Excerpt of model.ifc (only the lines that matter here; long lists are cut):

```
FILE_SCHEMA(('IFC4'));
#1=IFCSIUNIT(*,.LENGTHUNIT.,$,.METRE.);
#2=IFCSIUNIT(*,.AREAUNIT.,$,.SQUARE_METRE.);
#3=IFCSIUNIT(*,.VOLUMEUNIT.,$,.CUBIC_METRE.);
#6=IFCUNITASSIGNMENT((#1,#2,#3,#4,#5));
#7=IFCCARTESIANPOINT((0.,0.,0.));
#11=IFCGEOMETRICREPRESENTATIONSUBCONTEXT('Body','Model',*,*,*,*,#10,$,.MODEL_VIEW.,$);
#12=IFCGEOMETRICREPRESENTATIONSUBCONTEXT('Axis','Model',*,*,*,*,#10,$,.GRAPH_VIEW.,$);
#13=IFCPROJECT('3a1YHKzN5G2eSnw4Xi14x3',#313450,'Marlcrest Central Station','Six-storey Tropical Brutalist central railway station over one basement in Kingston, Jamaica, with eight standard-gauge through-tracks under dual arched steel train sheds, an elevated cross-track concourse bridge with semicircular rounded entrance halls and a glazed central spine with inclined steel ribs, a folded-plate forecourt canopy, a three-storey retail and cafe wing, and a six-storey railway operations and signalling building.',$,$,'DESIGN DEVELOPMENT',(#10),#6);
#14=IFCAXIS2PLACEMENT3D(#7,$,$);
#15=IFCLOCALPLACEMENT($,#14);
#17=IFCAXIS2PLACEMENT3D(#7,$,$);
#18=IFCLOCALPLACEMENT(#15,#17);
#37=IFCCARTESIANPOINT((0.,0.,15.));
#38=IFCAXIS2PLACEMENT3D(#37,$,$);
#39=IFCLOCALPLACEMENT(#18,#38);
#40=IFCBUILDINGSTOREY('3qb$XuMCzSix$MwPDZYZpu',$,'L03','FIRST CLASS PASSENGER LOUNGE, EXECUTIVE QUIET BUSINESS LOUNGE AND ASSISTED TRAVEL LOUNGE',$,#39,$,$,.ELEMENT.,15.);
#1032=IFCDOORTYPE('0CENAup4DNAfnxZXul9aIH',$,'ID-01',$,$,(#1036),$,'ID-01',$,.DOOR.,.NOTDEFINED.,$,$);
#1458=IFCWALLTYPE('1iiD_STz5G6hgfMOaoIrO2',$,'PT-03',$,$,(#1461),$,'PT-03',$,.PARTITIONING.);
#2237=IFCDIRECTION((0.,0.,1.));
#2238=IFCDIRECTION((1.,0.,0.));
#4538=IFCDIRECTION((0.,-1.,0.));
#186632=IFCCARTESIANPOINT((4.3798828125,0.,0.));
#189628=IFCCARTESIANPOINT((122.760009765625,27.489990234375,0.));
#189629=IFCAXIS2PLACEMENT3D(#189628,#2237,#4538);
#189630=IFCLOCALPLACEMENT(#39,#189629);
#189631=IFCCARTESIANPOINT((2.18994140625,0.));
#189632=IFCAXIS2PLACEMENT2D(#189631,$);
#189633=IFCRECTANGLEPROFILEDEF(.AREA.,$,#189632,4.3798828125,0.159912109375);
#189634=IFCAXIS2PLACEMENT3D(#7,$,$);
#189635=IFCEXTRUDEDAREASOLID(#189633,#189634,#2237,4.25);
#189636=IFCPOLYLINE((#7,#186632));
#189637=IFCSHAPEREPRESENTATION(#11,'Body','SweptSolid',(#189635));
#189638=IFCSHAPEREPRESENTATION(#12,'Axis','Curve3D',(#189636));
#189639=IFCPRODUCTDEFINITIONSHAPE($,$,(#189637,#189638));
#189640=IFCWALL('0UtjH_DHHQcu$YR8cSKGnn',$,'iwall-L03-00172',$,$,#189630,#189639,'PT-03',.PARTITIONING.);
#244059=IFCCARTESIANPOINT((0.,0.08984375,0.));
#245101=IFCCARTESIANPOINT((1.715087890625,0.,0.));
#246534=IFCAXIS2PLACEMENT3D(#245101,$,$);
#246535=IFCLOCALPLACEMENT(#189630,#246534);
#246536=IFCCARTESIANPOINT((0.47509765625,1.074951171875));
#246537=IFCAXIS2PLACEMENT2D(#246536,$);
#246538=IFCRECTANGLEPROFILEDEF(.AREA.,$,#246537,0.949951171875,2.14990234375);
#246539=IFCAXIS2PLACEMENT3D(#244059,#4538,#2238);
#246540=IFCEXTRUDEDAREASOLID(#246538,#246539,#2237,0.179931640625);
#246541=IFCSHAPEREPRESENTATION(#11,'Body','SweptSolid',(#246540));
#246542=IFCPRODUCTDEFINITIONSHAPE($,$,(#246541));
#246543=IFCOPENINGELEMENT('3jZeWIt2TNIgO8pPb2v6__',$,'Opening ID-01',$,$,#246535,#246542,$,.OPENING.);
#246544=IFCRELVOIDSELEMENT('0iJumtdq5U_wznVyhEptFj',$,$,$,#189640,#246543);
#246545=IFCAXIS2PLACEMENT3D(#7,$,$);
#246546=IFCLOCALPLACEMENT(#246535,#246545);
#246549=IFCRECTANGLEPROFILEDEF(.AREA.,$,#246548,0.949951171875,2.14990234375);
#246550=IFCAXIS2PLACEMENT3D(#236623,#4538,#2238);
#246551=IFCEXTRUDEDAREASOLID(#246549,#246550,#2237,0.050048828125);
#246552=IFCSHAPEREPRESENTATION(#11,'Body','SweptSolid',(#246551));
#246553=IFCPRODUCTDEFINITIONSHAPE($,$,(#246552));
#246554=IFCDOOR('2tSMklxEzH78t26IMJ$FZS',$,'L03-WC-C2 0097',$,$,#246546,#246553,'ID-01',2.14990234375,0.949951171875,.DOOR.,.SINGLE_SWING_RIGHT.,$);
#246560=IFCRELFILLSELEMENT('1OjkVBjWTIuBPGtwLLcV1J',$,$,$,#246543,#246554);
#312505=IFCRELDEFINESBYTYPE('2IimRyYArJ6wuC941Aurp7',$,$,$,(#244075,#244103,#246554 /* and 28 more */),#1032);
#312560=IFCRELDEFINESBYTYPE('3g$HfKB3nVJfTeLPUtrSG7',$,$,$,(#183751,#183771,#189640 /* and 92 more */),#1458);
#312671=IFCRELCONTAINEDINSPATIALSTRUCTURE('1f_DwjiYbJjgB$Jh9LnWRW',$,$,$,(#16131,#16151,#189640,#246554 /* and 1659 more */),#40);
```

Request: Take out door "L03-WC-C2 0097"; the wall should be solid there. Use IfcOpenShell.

```python
import ifcopenshell
import ifcopenshell.api.feature
import ifcopenshell.api.root
import ifcopenshell.geom
import ifcopenshell.util.shape

model = ifcopenshell.open("model.ifc")
settings = ifcopenshell.geom.settings()


def volume(element):
    """Net volume in cubic metres, openings subtracted."""
    shape = ifcopenshell.geom.create_shape(settings, element)
    return ifcopenshell.util.shape.get_volume(shape.geometry)


door = model.by_id(246554)
opening = door.FillsVoids[0].RelatingOpeningElement
wall = opening.VoidsElements[0].RelatingBuildingElement
before = volume(wall)

ifcopenshell.api.root.remove_product(model, product=door)
ifcopenshell.api.feature.remove_feature(model, feature=opening)

after = volume(wall)

print(f"wall volume {before:.3f} -> {after:.3f} m3")

model.write("model_v2.ifc")
```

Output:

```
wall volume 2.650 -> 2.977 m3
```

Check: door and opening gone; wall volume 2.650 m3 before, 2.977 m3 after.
